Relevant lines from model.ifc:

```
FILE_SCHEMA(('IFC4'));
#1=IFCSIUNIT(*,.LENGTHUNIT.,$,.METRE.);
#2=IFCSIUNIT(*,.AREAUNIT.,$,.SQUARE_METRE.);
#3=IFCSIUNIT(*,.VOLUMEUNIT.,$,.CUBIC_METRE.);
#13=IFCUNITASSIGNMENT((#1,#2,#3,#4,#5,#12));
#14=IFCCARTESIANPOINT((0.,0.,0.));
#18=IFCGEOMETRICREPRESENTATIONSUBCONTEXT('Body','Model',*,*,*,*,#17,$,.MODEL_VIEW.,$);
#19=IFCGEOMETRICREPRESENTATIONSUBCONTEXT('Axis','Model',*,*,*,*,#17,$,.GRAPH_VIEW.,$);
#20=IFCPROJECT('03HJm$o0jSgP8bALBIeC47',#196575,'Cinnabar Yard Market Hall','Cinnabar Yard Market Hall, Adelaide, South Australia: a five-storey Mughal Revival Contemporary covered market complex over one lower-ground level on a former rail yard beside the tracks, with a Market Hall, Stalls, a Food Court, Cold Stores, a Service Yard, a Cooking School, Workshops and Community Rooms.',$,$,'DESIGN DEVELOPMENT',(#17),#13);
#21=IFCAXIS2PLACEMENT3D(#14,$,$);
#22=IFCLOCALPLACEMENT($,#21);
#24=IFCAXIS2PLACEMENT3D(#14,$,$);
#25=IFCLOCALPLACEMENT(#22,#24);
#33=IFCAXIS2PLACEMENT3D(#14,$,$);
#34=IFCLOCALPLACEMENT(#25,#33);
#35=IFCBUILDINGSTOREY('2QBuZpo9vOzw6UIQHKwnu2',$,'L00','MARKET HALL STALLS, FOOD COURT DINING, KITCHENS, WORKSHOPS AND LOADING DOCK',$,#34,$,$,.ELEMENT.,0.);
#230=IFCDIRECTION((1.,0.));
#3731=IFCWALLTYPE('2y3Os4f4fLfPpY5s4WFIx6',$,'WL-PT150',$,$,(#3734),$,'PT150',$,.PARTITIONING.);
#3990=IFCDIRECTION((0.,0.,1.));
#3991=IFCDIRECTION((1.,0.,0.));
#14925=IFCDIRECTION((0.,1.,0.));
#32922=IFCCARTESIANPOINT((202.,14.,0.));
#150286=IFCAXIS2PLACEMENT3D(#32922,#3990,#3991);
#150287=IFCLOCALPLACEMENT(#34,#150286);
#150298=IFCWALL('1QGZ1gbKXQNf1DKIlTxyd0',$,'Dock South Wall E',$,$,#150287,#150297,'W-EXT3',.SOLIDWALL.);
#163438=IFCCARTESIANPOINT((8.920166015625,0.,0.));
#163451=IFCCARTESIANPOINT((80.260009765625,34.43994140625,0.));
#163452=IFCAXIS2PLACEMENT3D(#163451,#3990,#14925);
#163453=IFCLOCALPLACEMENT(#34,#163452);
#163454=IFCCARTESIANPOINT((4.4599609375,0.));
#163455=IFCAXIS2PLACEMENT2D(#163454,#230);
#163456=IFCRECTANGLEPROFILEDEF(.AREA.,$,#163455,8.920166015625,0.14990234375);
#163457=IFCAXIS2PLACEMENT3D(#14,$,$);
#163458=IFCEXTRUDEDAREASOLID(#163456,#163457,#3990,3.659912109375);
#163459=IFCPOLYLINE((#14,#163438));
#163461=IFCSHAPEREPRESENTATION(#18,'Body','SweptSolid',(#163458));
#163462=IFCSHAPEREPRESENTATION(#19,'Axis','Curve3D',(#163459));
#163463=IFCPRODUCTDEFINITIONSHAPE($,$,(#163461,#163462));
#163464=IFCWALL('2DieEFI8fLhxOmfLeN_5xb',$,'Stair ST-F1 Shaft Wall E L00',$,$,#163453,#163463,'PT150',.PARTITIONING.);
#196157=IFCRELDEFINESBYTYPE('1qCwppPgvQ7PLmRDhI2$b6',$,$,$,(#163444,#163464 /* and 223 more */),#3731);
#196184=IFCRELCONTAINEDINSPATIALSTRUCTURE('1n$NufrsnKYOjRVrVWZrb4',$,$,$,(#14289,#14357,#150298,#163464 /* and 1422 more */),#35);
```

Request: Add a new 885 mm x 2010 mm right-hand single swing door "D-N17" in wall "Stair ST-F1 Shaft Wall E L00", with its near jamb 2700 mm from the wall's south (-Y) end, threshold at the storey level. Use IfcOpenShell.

```python
import numpy as np
import ifcopenshell
import ifcopenshell.api.feature
import ifcopenshell.api.geometry
import ifcopenshell.api.root
import ifcopenshell.api.spatial
import ifcopenshell.geom
import ifcopenshell.util.element
import ifcopenshell.util.placement
import ifcopenshell.util.representation
import ifcopenshell.util.shape
import ifcopenshell.util.unit

model = ifcopenshell.open("model.ifc")
unit_scale = ifcopenshell.util.unit.calculate_unit_scale(model)
settings = ifcopenshell.geom.settings()


def volume(element):
    """Net volume in cubic metres, openings subtracted."""
    shape = ifcopenshell.geom.create_shape(settings, element)
    return ifcopenshell.util.shape.get_volume(shape.geometry)


wall = model.by_id(163464)
storey = ifcopenshell.util.element.get_container(wall, ifc_class="IfcBuildingStorey")
context = ifcopenshell.util.representation.get_context(model, "Model", "Body", "MODEL_VIEW")
before = volume(wall)

width, height, from_end, sill = 0.885, 2.01, 2.7, 0.0  # metres

# The wall runs along its own X axis, and the end named is its -X end.
wall_shape = ifcopenshell.geom.create_shape(settings, wall)
x, y, z = ifcopenshell.util.shape.get_vertices(wall_shape.geometry).T
start = x.min() + from_end
face, thickness = float(y.min()), float(y.max() - y.min())
wall_matrix = ifcopenshell.util.placement.get_local_placement(wall.ObjectPlacement)
level = ifcopenshell.util.placement.get_local_placement(storey.ObjectPlacement)[2, 3]


def in_wall(x, y):
    """Placement at x, y metres in the wall's axes, at sill height."""
    matrix = wall_matrix.copy()
    matrix[:, 3] = wall_matrix @ np.array([x / unit_scale, y / unit_scale, 0.0, 1.0])
    matrix[2, 3] = level + sill / unit_scale
    return matrix


# Opening: a box that overshoots both wall faces by 50 mm.
opening = ifcopenshell.api.root.create_entity(model, ifc_class="IfcOpeningElement", predefined_type="OPENING")
box = ifcopenshell.api.geometry.add_wall_representation(
    model, context=context, length=width, height=height, thickness=thickness + 0.1
)
ifcopenshell.api.geometry.assign_representation(model, product=opening, representation=box)
ifcopenshell.api.geometry.edit_object_placement(model, product=opening, matrix=in_wall(start, face - 0.05), is_si=False)
ifcopenshell.api.feature.add_feature(model, feature=opening, element=wall)

door = ifcopenshell.api.root.create_entity(model, ifc_class="IfcDoor", name="D-N17", predefined_type="DOOR")
door.OverallWidth, door.OverallHeight = width / unit_scale, height / unit_scale
door.OperationType = "SINGLE_SWING_RIGHT"
body = ifcopenshell.api.geometry.add_door_representation(
    model,
    context=context,
    overall_width=door.OverallWidth,
    overall_height=door.OverallHeight,
    operation_type="SINGLE_SWING_RIGHT",
    lining_properties={"LiningDepth": thickness / unit_scale, "ThresholdDepth": thickness / unit_scale},
)
ifcopenshell.api.geometry.assign_representation(model, product=door, representation=body)
ifcopenshell.api.spatial.assign_container(model, products=[door], relating_structure=storey)
ifcopenshell.api.feature.add_filling(model, opening=opening, element=door)

# The lining spans the wall, so the door starts at the wall face.
ifcopenshell.api.geometry.edit_object_placement(model, product=door, matrix=in_wall(start, face), is_si=False)

after = volume(wall)

print(f"wall volume {before:.3f} -> {after:.3f} m3")

model.write("model_updated.ifc")
```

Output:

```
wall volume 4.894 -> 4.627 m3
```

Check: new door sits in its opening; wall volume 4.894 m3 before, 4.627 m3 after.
